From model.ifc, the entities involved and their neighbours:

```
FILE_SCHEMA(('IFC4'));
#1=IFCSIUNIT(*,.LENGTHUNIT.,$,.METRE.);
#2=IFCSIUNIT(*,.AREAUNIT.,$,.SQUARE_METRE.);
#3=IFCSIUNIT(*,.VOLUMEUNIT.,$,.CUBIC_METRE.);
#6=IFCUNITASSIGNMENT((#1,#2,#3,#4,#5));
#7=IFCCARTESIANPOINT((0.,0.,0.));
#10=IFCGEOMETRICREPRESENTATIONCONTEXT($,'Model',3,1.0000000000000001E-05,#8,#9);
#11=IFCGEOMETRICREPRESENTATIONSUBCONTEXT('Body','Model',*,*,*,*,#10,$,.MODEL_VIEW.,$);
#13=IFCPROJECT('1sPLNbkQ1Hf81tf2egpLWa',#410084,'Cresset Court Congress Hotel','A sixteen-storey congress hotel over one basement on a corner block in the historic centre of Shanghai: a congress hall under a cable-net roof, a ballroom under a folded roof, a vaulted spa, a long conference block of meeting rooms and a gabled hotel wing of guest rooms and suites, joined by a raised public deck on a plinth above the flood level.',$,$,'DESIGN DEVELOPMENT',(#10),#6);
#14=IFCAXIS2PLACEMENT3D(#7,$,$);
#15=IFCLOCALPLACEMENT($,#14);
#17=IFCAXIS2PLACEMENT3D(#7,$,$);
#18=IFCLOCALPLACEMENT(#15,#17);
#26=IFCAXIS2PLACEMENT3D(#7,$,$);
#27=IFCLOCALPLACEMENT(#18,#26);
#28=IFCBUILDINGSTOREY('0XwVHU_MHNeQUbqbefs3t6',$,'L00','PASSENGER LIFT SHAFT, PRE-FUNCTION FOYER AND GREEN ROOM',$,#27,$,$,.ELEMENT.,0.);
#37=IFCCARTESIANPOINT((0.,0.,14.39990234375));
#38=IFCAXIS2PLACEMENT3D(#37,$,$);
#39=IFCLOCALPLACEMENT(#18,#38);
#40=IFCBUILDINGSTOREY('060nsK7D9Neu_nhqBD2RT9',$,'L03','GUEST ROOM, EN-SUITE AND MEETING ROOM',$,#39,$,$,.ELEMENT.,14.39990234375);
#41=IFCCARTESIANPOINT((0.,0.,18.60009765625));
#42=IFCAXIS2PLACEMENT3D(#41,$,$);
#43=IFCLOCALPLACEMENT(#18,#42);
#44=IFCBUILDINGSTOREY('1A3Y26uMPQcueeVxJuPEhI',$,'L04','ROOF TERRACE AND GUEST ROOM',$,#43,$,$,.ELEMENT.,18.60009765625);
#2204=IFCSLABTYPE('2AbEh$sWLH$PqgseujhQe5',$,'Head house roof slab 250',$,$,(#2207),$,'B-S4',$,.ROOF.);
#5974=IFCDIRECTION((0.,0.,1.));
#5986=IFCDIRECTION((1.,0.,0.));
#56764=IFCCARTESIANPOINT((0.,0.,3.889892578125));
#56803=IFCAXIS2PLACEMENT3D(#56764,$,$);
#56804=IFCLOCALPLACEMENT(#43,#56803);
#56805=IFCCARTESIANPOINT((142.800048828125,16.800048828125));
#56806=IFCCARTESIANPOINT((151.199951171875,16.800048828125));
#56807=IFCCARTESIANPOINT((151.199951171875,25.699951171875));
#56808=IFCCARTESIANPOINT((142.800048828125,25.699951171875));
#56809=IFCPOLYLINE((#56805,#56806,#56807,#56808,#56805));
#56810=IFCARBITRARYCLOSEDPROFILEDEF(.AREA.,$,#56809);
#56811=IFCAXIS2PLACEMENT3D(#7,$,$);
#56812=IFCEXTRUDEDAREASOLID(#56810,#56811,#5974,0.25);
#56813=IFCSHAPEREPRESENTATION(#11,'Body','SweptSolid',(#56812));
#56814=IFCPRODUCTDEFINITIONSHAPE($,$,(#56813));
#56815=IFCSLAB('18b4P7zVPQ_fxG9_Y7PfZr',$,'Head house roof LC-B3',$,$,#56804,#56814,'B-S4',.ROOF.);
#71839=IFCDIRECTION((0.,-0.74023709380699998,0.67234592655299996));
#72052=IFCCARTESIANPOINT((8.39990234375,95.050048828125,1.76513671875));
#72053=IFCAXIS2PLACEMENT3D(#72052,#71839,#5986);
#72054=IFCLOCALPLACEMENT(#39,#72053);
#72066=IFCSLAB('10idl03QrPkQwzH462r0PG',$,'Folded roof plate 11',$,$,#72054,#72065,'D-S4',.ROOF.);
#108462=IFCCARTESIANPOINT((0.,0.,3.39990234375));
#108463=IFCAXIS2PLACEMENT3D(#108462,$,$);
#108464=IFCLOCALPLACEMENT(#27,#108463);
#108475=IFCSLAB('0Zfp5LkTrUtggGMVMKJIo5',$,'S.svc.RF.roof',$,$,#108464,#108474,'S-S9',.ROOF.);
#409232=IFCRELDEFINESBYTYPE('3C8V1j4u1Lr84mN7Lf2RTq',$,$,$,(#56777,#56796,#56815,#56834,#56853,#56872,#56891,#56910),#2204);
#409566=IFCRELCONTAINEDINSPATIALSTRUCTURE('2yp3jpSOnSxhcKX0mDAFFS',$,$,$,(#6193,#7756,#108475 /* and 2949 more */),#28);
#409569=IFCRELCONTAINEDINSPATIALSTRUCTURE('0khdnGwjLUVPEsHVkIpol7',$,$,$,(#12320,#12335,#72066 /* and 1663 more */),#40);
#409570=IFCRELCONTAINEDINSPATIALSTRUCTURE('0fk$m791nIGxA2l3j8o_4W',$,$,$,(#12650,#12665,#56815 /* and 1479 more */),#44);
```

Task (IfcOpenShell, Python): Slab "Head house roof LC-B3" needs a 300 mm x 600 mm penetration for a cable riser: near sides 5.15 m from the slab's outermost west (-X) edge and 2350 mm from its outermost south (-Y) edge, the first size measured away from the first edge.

```python
import numpy as np
import ifcopenshell
import ifcopenshell.api.feature
import ifcopenshell.api.geometry
import ifcopenshell.api.root
import ifcopenshell.geom
import ifcopenshell.util.placement
import ifcopenshell.util.representation
import ifcopenshell.util.shape
import ifcopenshell.util.unit

model = ifcopenshell.open("model.ifc")
unit_scale = ifcopenshell.util.unit.calculate_unit_scale(model)
settings = ifcopenshell.geom.settings()


def volume(element):
    """Net volume in cubic metres, openings subtracted."""
    shape = ifcopenshell.geom.create_shape(settings, element)
    return ifcopenshell.util.shape.get_volume(shape.geometry)


slab = model.by_guid("18b4P7zVPQ_fxG9_Y7PfZr")
before = volume(slab)

# Extent in the slab's own axes, in metres. The edges named are its -X and -Y sides.
slab_shape = ifcopenshell.geom.create_shape(settings, slab)
vertices = ifcopenshell.util.shape.get_vertices(slab_shape.geometry)
x_min, y_min, bottom = vertices.min(axis=0)
top = vertices[:, 2].max()

opening = ifcopenshell.api.root.create_entity(model, ifc_class="IfcOpeningElement", name="Cable riser opening", predefined_type="OPENING")
context = ifcopenshell.util.representation.get_context(model, "Model", "Body", "MODEL_VIEW")
width, depth = 0.3, 0.6
outline = [(0.0, 0.0), (width, 0.0), (width, depth), (0.0, depth), (0.0, 0.0)]
# Overshoot both faces by 50 mm so the cut is clean.
shape = ifcopenshell.api.geometry.add_slab_representation(
    model, context=context, depth=top - bottom + 0.1, polyline=outline
)
ifcopenshell.api.geometry.assign_representation(model, product=opening, representation=shape)

matrix = ifcopenshell.util.placement.get_local_placement(slab.ObjectPlacement)
matrix[:, 3] = matrix @ np.append(np.array([x_min + 5.15, y_min + 2.35, bottom - 0.05]) / unit_scale, 1.0)
ifcopenshell.api.geometry.edit_object_placement(model, product=opening, matrix=matrix, is_si=False)
ifcopenshell.api.feature.add_feature(model, feature=opening, element=slab)

after = volume(slab)

print(f"slab volume {before:.3f} -> {after:.3f} m3")

model.write("model_updated.ifc")
```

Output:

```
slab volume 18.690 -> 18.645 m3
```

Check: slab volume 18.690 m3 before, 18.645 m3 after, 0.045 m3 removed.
